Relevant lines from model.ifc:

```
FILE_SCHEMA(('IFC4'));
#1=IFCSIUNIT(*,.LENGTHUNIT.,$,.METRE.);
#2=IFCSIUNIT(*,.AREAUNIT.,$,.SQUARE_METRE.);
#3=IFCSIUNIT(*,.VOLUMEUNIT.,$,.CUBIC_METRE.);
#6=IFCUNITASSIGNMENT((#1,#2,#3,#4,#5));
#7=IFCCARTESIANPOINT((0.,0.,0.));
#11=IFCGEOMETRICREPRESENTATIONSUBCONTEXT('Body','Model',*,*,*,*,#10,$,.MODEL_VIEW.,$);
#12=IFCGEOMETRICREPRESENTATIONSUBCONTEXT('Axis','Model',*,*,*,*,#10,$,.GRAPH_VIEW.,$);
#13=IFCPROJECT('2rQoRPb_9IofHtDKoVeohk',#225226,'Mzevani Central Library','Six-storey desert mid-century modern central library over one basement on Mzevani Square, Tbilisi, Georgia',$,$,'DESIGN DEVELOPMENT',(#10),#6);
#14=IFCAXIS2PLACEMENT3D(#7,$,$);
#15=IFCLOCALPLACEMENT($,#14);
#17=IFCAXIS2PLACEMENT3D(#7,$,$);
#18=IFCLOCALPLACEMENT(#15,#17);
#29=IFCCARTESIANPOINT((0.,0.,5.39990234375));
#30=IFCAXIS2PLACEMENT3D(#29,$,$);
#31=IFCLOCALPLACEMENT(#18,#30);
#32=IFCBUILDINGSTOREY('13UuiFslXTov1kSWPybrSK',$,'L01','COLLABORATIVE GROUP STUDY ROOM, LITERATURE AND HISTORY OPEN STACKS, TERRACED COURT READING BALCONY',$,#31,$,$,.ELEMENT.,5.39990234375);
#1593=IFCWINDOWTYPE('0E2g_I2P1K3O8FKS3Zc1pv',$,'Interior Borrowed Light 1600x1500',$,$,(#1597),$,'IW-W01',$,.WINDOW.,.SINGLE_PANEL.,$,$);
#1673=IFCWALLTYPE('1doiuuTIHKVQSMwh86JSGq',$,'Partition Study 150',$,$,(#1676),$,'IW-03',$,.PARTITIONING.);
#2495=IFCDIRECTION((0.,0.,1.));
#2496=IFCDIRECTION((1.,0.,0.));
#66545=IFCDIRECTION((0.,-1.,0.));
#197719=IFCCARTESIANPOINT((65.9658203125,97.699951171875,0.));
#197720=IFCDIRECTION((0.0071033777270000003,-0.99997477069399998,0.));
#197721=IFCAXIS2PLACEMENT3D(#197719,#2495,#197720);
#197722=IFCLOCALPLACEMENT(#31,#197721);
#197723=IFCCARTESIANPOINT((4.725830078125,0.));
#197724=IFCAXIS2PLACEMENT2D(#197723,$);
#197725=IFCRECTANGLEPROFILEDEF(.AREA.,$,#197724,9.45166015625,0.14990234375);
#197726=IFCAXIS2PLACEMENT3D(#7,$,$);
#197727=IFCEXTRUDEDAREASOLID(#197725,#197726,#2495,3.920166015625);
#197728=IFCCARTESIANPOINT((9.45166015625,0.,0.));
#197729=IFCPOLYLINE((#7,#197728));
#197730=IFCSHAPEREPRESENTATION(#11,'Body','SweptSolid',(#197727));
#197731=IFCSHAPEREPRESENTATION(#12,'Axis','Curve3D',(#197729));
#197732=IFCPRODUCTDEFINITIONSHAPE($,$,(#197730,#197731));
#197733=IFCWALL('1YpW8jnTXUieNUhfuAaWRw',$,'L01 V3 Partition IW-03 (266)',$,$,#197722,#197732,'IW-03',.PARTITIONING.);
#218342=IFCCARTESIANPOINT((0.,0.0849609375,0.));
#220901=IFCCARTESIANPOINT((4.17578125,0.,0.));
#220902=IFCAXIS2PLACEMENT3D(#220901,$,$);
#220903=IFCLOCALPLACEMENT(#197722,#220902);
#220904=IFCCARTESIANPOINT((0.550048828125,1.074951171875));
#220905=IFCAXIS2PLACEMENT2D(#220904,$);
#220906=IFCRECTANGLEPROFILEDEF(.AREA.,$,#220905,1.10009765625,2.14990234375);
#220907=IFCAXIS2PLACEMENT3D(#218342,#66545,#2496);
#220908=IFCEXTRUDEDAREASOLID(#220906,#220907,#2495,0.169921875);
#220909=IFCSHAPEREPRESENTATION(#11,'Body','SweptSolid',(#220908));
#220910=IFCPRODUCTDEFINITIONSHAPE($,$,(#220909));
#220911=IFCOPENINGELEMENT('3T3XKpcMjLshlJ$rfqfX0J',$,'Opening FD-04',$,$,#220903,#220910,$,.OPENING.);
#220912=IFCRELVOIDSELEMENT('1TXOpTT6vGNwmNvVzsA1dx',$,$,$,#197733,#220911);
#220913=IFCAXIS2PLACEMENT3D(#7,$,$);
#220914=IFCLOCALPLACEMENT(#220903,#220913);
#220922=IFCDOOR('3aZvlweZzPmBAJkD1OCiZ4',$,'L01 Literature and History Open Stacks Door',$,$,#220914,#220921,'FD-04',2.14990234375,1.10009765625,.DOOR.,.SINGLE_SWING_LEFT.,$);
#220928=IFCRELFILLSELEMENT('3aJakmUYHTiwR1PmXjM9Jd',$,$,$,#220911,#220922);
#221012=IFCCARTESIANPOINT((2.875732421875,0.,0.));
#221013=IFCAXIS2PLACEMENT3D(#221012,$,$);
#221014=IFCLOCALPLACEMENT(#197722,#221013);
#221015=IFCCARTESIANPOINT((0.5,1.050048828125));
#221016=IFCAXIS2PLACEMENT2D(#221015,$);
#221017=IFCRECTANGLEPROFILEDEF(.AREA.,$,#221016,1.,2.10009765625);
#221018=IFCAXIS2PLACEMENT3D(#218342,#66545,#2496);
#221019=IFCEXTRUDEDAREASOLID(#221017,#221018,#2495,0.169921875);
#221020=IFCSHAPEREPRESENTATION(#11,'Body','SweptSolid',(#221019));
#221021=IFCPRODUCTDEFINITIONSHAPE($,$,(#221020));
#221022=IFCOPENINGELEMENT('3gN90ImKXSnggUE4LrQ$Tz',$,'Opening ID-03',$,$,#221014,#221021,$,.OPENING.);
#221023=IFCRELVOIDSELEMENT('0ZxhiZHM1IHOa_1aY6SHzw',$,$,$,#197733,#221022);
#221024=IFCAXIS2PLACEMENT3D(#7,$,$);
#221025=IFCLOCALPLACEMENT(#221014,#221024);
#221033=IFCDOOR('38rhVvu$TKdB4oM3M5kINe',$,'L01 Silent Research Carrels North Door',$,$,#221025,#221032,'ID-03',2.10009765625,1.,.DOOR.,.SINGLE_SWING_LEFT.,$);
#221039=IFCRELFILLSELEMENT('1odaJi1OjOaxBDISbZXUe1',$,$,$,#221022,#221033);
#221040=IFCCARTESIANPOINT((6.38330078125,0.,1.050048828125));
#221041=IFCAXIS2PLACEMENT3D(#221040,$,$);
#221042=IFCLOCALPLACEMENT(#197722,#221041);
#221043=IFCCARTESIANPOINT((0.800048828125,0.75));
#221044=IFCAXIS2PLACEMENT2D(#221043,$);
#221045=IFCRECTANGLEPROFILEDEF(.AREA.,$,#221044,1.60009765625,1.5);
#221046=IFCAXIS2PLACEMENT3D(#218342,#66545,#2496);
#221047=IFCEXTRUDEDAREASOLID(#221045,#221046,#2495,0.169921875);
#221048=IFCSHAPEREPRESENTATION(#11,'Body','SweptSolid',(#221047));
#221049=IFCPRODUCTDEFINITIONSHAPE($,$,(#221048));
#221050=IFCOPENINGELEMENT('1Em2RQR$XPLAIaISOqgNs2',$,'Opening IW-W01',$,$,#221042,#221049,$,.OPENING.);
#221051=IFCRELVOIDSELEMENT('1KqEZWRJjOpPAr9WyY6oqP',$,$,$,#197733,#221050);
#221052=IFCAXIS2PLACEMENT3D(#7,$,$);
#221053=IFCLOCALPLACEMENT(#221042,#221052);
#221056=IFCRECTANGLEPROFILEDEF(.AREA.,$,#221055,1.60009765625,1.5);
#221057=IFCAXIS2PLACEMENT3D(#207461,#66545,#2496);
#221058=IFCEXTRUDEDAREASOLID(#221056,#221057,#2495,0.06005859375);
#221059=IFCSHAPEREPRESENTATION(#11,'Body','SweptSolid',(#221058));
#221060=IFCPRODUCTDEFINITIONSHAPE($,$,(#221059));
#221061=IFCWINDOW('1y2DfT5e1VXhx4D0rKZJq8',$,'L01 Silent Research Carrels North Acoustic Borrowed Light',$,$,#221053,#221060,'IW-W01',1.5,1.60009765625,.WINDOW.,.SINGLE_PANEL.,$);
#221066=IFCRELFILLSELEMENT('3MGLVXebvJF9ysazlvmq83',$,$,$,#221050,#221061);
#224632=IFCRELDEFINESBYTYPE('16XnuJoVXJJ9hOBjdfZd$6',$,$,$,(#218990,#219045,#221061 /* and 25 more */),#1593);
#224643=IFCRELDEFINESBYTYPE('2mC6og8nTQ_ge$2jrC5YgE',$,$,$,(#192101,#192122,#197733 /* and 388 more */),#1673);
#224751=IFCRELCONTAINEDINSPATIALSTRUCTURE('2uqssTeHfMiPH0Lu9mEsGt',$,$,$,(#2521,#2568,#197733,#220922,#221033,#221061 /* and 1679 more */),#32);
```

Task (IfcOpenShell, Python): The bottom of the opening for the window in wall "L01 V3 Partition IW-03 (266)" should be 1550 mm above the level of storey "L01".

```python
import numpy as np
import ifcopenshell
import ifcopenshell.api.geometry
import ifcopenshell.geom
import ifcopenshell.util.element
import ifcopenshell.util.placement
import ifcopenshell.util.shape
import ifcopenshell.util.unit

model = ifcopenshell.open("model.ifc")
unit_scale = ifcopenshell.util.unit.calculate_unit_scale(model)

window = model.by_id(221061)
opening = window.FillsVoids[0].RelatingOpeningElement
storey = ifcopenshell.util.element.get_container(window, ifc_class="IfcBuildingStorey")
level = ifcopenshell.util.placement.get_local_placement(storey.ObjectPlacement)[2, 3]

# The opening's origin need not be at the sill, so measure its lowest point.
shape = ifcopenshell.geom.create_shape(ifcopenshell.geom.settings(), opening)
bottom = ifcopenshell.util.shape.get_shape_bottom_elevation(shape, shape.geometry) / unit_scale
dz = level + 1.55 - bottom

shift = np.array([0.0, 0.0, dz])
# The window is placed relative to its opening, so it follows when the opening moves.
matrix = ifcopenshell.util.placement.get_local_placement(opening.ObjectPlacement)
matrix[:3, 3] += shift
ifcopenshell.api.geometry.edit_object_placement(
    model, product=opening, matrix=matrix, is_si=False, should_transform_children=True
)

print(f"moved by {dz * unit_scale:+.3f} m")

model.write("model-out.ifc")
```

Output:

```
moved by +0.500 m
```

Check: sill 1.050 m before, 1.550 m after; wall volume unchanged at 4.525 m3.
